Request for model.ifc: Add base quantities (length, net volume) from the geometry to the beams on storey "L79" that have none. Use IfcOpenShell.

First a look at what the model holds.

```python
import ifcopenshell
import ifcopenshell.util.element
import ifcopenshell.util.unit

model = ifcopenshell.open("model.ifc")
print(model.schema)
for unit_type in ("LENGTHUNIT", "AREAUNIT", "VOLUMEUNIT"):
    print(unit_type, ifcopenshell.util.unit.calculate_unit_scale(model, unit_type))
storey = next(s for s in model.by_type("IfcBuildingStorey") if s.Name == "L79")
beams = [e for e in ifcopenshell.util.element.get_decomposition(storey) if e.is_a("IfcBeam")]
for e in sorted(beams, key=lambda e: e.id()):
    print(e.id(), e.is_a(), e.Name, list(ifcopenshell.util.element.get_psets(e, qtos_only=True)), sep=" | ")
```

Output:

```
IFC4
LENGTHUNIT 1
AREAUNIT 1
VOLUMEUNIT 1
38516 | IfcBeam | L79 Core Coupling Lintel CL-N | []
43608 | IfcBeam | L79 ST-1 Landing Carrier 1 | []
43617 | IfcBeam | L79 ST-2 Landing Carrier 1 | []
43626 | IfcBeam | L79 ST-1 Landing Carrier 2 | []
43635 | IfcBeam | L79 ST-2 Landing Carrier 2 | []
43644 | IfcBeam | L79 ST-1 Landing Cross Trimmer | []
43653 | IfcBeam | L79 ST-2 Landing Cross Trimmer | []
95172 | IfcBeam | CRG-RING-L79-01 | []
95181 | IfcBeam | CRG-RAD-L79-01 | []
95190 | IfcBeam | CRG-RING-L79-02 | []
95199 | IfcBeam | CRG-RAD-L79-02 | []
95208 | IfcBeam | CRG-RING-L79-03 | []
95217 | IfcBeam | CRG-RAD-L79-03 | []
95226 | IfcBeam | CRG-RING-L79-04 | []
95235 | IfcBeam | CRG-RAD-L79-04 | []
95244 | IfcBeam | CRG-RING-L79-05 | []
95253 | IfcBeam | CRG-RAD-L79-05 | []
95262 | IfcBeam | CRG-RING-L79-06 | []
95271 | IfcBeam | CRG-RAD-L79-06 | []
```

```python
import ifcopenshell
import ifcopenshell.api.pset
import ifcopenshell.geom
import ifcopenshell.util.element
import ifcopenshell.util.shape
import ifcopenshell.util.unit

model = ifcopenshell.open("model.ifc")
unit_scale = ifcopenshell.util.unit.calculate_unit_scale(model)
volume_scale = ifcopenshell.util.unit.calculate_unit_scale(model, "VOLUMEUNIT")
settings = ifcopenshell.geom.settings()

storey = next(s for s in model.by_type("IfcBuildingStorey") if s.Name == "L79")
beams = [e for e in ifcopenshell.util.element.get_decomposition(storey) if e.is_a("IfcBeam")]

for e in sorted(beams, key=lambda e: e.id()):
    if ifcopenshell.util.element.get_psets(e, qtos_only=True, should_inherit=False):
        continue
    # Geometry comes back in metres, in the element's own axes.
    shape = ifcopenshell.geom.create_shape(settings, e)
    values = {
        "Length": ifcopenshell.util.shape.get_max_xyz(shape.geometry) / unit_scale,
        "NetVolume": ifcopenshell.util.shape.get_volume(shape.geometry) / volume_scale,
    }
    qto = ifcopenshell.api.pset.add_qto(model, product=e, name="Qto_BeamBaseQuantities")
    ifcopenshell.api.pset.edit_qto(model, qto=qto, properties=values)
    print(e.id(), {k: round(v, 3) for k, v in values.items()})

model.write("model_rev.ifc")
```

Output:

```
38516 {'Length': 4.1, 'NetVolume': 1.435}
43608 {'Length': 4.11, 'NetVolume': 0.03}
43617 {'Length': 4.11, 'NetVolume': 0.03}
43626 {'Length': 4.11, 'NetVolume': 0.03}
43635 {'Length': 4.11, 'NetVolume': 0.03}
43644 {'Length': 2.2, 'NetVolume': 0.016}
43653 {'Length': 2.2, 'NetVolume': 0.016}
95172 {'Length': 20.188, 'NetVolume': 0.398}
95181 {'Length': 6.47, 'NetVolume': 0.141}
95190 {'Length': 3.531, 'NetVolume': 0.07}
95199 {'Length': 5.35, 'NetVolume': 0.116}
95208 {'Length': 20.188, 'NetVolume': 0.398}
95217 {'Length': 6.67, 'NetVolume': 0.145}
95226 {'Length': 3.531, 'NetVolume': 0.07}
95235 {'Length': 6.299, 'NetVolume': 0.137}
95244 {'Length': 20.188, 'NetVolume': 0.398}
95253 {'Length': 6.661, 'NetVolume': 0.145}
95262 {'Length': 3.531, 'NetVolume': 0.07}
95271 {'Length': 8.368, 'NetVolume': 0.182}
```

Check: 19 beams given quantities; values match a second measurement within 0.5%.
